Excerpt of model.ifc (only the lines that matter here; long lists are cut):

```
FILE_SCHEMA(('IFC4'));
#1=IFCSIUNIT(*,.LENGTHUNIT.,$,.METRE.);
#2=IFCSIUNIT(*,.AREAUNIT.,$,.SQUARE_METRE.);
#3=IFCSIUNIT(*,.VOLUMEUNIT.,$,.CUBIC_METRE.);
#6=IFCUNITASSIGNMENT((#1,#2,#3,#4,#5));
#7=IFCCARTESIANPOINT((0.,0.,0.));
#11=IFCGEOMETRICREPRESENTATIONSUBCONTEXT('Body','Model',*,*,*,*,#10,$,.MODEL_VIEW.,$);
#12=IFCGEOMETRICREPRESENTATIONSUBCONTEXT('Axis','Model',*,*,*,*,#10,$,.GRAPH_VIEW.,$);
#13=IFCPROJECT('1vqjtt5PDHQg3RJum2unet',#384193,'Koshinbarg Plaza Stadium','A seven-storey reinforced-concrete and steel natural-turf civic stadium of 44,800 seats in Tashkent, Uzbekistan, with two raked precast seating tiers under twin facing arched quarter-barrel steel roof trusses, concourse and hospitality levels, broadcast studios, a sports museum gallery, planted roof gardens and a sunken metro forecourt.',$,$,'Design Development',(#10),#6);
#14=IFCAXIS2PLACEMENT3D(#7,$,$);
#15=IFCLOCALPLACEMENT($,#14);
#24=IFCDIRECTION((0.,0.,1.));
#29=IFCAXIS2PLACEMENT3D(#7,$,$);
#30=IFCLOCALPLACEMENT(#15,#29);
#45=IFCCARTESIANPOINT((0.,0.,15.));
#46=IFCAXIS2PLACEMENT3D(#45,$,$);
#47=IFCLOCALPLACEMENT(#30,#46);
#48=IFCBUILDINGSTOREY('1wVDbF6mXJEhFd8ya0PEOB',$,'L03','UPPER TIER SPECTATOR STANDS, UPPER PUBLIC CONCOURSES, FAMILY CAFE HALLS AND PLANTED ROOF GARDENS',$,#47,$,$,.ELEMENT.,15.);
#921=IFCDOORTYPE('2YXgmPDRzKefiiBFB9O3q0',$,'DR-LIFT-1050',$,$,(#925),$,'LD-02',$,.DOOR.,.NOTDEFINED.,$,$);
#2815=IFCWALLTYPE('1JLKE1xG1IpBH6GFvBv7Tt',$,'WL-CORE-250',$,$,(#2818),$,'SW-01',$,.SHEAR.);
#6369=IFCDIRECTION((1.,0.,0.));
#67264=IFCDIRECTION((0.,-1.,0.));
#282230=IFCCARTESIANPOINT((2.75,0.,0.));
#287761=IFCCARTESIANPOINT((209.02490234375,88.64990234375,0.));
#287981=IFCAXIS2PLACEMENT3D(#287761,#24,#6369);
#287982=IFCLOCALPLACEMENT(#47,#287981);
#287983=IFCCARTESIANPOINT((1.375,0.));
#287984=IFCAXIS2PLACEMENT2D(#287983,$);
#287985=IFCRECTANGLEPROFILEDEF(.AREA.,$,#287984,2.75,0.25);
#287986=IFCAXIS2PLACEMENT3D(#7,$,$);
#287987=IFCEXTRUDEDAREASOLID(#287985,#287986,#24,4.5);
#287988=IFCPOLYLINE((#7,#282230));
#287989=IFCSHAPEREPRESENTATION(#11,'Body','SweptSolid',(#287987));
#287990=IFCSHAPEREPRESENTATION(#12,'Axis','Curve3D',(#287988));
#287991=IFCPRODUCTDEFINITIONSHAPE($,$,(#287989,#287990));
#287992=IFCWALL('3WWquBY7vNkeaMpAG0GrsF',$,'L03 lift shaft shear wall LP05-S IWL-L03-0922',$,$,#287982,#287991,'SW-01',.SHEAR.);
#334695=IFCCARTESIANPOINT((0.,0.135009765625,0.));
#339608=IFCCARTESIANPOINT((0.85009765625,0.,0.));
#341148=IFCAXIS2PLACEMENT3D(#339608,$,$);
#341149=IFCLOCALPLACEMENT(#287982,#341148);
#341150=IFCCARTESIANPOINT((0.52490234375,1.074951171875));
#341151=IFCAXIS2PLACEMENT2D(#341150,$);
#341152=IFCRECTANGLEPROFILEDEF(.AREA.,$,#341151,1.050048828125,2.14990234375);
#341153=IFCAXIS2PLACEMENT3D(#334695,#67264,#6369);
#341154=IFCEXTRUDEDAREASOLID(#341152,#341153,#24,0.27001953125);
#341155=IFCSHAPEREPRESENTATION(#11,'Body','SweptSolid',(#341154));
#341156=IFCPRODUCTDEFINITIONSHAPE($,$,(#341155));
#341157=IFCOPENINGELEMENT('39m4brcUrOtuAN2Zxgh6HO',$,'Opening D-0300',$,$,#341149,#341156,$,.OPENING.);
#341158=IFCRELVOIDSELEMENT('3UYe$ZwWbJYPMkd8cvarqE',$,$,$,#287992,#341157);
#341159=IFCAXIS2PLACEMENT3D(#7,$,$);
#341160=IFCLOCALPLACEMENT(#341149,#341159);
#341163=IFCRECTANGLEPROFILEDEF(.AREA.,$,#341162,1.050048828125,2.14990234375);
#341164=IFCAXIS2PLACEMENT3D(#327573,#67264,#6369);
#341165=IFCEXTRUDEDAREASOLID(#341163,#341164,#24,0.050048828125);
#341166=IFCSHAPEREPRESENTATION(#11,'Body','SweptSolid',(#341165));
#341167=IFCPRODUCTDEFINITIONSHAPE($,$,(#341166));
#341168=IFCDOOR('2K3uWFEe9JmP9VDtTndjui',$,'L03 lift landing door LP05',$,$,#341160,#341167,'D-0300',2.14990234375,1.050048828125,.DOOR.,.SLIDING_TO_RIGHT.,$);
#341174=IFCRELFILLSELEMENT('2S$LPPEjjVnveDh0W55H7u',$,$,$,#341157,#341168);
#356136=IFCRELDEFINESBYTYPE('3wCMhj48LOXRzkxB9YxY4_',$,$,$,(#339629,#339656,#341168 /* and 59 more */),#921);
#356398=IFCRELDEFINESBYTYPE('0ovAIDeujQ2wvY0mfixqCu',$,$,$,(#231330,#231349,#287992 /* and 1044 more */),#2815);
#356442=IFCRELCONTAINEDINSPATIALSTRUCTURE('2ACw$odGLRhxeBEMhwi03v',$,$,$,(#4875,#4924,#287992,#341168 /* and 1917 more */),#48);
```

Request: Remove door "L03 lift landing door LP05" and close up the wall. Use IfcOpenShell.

```python
import ifcopenshell
import ifcopenshell.api.feature
import ifcopenshell.api.root
import ifcopenshell.geom
import ifcopenshell.util.shape

model = ifcopenshell.open("model.ifc")
settings = ifcopenshell.geom.settings()


def volume(element):
    """Net volume in cubic metres, openings subtracted."""
    shape = ifcopenshell.geom.create_shape(settings, element)
    return ifcopenshell.util.shape.get_volume(shape.geometry)


door = model.by_guid("2K3uWFEe9JmP9VDtTndjui")
opening = door.FillsVoids[0].RelatingOpeningElement
wall = opening.VoidsElements[0].RelatingBuildingElement
before = volume(wall)

ifcopenshell.api.root.remove_product(model, product=door)
ifcopenshell.api.feature.remove_feature(model, feature=opening)

after = volume(wall)

print(f"wall volume {before:.3f} -> {after:.3f} m3")

model.write("model_rev.ifc")
```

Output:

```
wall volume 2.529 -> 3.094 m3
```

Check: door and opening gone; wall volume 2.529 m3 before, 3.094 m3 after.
